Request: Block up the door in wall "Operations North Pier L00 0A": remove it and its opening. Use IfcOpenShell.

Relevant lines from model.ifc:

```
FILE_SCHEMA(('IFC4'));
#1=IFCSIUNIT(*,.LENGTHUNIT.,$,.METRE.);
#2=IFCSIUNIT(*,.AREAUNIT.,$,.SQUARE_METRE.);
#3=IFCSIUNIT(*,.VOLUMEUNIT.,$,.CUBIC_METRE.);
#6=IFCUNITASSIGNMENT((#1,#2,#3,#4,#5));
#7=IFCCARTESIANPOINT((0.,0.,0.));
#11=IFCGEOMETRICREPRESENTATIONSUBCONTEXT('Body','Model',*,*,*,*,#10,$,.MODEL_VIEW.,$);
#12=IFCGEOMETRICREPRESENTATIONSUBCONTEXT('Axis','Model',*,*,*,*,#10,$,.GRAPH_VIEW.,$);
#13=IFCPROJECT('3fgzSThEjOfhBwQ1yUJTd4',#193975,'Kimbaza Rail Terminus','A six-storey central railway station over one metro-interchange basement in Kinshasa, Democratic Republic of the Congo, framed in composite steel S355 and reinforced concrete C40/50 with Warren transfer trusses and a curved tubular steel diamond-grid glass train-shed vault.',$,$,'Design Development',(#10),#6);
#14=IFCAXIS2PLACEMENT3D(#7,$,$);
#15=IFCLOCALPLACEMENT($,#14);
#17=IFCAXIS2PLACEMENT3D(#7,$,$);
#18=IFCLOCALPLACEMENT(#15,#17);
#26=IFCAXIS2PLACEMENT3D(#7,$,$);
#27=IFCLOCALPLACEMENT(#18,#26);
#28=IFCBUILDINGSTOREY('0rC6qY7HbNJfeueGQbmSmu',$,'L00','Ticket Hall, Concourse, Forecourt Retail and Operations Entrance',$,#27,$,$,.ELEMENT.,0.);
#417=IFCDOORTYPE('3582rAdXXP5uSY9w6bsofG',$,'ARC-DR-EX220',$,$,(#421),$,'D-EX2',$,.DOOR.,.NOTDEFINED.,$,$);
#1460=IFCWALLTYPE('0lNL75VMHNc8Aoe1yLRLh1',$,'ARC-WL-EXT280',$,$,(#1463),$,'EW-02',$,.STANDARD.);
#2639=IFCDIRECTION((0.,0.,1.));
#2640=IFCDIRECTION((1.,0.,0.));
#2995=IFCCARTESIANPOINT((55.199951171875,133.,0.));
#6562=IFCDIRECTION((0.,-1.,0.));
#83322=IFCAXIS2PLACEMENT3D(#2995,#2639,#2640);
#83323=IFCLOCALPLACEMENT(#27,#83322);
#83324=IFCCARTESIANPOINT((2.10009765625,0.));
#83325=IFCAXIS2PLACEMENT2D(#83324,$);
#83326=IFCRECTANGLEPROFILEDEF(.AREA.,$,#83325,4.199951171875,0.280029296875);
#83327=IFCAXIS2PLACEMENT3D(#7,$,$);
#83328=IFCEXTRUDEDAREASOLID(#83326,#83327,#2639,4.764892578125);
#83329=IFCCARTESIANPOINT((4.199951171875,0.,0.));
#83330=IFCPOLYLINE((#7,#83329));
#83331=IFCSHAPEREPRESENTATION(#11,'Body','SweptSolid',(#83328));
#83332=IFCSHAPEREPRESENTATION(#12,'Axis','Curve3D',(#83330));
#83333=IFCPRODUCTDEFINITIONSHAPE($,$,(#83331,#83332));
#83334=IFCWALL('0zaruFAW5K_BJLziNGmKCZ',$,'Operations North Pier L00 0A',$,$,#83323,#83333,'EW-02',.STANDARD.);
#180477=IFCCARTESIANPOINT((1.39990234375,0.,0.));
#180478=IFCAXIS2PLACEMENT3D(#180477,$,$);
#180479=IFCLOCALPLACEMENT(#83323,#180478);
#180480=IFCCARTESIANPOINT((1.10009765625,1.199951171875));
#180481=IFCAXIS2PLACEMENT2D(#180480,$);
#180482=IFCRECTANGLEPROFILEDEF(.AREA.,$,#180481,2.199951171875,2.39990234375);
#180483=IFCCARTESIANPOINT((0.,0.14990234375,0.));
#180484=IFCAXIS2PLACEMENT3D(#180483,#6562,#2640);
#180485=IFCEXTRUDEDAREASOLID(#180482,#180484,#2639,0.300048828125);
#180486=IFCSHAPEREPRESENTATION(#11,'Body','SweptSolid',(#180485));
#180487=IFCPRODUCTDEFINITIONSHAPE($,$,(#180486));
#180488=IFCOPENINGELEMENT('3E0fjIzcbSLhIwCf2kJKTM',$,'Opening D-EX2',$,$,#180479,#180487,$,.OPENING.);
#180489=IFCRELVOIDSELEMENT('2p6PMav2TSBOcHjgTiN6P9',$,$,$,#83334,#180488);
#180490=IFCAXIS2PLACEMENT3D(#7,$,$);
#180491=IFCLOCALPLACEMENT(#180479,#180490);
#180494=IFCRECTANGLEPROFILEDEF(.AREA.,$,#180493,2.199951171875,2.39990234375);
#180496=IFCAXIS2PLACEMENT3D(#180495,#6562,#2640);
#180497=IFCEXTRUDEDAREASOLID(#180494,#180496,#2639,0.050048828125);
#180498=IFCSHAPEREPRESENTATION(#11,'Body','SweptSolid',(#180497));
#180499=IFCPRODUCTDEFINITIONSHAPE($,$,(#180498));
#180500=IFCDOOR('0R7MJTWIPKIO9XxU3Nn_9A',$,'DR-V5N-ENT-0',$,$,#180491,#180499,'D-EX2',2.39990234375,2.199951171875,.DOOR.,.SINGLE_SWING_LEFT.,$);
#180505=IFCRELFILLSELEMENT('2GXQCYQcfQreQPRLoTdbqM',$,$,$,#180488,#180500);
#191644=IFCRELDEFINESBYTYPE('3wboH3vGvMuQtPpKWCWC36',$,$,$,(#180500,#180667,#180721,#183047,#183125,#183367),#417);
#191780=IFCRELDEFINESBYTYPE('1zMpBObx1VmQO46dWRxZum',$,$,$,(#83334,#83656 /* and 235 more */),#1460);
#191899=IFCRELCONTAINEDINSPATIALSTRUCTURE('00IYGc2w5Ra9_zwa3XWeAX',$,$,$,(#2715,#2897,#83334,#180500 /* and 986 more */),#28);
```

```python
import ifcopenshell
import ifcopenshell.api.feature
import ifcopenshell.api.root
import ifcopenshell.geom
import ifcopenshell.util.shape

model = ifcopenshell.open("model.ifc")
settings = ifcopenshell.geom.settings()


def volume(element):
    """Net volume in cubic metres, openings subtracted."""
    shape = ifcopenshell.geom.create_shape(settings, element)
    return ifcopenshell.util.shape.get_volume(shape.geometry)


door = model.by_id(180500)
opening = door.FillsVoids[0].RelatingOpeningElement
wall = opening.VoidsElements[0].RelatingBuildingElement
before = volume(wall)

ifcopenshell.api.root.remove_product(model, product=door)
ifcopenshell.api.feature.remove_feature(model, feature=opening)

after = volume(wall)

print(f"wall volume {before:.3f} -> {after:.3f} m3")

model.write("model_updated.ifc")
```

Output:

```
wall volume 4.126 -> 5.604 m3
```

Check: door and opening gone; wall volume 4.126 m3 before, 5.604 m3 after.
